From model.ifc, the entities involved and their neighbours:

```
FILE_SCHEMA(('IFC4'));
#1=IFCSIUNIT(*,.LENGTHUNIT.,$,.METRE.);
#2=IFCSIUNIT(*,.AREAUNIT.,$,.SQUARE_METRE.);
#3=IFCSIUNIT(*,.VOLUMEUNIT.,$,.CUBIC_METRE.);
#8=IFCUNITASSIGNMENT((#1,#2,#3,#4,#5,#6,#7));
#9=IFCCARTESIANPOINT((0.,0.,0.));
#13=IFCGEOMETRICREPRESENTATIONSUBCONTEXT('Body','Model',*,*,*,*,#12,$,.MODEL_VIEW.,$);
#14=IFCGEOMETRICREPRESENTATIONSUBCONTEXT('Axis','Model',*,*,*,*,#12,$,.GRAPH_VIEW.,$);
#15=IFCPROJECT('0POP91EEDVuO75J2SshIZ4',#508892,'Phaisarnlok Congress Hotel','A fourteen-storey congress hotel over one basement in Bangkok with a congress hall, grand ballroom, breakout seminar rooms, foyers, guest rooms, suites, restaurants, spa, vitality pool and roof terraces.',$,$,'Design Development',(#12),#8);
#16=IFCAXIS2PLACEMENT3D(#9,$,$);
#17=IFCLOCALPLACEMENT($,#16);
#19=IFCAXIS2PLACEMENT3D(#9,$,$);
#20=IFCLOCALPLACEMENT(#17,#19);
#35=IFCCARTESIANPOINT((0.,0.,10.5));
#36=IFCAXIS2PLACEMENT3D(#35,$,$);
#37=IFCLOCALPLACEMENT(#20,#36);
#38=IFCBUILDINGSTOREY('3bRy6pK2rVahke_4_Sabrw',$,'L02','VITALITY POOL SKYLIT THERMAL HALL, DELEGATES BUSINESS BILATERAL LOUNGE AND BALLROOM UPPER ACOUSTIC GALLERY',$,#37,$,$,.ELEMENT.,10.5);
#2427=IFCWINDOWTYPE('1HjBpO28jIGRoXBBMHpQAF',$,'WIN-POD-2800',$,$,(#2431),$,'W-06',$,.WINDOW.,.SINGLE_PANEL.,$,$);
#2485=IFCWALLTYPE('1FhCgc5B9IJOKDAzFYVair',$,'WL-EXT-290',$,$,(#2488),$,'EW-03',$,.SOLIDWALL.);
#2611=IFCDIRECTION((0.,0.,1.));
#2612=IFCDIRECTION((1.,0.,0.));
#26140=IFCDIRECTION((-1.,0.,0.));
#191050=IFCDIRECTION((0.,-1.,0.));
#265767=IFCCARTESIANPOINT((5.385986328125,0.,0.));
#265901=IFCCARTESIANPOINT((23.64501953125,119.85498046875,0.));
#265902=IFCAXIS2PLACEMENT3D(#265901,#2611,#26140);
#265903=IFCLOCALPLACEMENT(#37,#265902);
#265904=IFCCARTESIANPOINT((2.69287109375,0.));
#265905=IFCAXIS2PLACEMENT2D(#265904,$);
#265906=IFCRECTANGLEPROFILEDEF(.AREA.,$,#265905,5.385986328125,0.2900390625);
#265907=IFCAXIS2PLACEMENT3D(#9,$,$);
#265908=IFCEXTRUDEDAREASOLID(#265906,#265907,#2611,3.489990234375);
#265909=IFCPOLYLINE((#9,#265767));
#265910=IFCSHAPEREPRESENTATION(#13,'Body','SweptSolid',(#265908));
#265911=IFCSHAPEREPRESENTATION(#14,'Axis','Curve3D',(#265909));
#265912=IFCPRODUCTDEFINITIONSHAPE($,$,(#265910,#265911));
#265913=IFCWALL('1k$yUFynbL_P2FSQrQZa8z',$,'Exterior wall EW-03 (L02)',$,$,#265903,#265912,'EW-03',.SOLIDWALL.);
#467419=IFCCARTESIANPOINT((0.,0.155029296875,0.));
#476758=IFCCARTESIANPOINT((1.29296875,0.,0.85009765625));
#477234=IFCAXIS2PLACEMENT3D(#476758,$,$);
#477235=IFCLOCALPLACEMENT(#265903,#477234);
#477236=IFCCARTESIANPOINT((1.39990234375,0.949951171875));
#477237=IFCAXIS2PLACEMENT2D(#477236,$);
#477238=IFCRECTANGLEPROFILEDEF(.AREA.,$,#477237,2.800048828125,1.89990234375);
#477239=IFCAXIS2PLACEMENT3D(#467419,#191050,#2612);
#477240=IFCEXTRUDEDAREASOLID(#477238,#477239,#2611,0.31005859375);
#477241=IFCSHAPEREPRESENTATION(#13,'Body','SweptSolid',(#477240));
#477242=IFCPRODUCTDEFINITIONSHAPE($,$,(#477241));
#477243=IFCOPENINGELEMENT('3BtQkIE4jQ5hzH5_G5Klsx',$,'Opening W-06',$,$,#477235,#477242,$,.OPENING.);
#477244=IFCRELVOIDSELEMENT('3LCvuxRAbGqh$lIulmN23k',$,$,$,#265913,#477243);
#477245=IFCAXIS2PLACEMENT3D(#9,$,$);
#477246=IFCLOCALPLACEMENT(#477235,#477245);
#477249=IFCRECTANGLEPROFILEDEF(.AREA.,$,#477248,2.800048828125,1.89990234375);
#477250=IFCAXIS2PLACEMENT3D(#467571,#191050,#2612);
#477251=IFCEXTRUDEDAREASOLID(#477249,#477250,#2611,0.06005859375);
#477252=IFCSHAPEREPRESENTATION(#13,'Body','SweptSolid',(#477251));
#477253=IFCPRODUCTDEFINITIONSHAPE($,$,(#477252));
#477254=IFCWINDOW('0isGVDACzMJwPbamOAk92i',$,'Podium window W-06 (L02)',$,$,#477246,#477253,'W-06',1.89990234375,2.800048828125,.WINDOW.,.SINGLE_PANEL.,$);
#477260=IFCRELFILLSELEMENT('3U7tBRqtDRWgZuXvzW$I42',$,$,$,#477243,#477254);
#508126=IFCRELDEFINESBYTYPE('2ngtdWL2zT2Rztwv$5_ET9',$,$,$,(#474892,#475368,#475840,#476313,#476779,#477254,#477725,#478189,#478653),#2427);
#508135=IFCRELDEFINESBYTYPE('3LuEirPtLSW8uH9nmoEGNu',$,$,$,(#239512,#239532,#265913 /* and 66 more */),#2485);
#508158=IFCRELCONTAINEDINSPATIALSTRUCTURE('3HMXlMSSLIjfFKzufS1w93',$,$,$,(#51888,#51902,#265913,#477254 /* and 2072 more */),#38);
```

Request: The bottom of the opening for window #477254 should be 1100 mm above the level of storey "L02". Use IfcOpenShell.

```python
import numpy as np
import ifcopenshell
import ifcopenshell.api.geometry
import ifcopenshell.geom
import ifcopenshell.util.element
import ifcopenshell.util.placement
import ifcopenshell.util.shape
import ifcopenshell.util.unit

model = ifcopenshell.open("model.ifc")
unit_scale = ifcopenshell.util.unit.calculate_unit_scale(model)

window = model.by_guid("0isGVDACzMJwPbamOAk92i")
opening = window.FillsVoids[0].RelatingOpeningElement
storey = ifcopenshell.util.element.get_container(window, ifc_class="IfcBuildingStorey")
level = ifcopenshell.util.placement.get_local_placement(storey.ObjectPlacement)[2, 3]

# The opening's origin need not be at the sill, so measure its lowest point.
shape = ifcopenshell.geom.create_shape(ifcopenshell.geom.settings(), opening)
bottom = ifcopenshell.util.shape.get_shape_bottom_elevation(shape, shape.geometry) / unit_scale
dz = level + 1.1 - bottom

shift = np.array([0.0, 0.0, dz])
# The window is placed relative to its opening, so it follows when the opening moves.
matrix = ifcopenshell.util.placement.get_local_placement(opening.ObjectPlacement)
matrix[:3, 3] += shift
ifcopenshell.api.geometry.edit_object_placement(
    model, product=opening, matrix=matrix, is_si=False, should_transform_children=True
)

print(f"moved by {dz * unit_scale:+.3f} m")

model.write("model-out.ifc")
```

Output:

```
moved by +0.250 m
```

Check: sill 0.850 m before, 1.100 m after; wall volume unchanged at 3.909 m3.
